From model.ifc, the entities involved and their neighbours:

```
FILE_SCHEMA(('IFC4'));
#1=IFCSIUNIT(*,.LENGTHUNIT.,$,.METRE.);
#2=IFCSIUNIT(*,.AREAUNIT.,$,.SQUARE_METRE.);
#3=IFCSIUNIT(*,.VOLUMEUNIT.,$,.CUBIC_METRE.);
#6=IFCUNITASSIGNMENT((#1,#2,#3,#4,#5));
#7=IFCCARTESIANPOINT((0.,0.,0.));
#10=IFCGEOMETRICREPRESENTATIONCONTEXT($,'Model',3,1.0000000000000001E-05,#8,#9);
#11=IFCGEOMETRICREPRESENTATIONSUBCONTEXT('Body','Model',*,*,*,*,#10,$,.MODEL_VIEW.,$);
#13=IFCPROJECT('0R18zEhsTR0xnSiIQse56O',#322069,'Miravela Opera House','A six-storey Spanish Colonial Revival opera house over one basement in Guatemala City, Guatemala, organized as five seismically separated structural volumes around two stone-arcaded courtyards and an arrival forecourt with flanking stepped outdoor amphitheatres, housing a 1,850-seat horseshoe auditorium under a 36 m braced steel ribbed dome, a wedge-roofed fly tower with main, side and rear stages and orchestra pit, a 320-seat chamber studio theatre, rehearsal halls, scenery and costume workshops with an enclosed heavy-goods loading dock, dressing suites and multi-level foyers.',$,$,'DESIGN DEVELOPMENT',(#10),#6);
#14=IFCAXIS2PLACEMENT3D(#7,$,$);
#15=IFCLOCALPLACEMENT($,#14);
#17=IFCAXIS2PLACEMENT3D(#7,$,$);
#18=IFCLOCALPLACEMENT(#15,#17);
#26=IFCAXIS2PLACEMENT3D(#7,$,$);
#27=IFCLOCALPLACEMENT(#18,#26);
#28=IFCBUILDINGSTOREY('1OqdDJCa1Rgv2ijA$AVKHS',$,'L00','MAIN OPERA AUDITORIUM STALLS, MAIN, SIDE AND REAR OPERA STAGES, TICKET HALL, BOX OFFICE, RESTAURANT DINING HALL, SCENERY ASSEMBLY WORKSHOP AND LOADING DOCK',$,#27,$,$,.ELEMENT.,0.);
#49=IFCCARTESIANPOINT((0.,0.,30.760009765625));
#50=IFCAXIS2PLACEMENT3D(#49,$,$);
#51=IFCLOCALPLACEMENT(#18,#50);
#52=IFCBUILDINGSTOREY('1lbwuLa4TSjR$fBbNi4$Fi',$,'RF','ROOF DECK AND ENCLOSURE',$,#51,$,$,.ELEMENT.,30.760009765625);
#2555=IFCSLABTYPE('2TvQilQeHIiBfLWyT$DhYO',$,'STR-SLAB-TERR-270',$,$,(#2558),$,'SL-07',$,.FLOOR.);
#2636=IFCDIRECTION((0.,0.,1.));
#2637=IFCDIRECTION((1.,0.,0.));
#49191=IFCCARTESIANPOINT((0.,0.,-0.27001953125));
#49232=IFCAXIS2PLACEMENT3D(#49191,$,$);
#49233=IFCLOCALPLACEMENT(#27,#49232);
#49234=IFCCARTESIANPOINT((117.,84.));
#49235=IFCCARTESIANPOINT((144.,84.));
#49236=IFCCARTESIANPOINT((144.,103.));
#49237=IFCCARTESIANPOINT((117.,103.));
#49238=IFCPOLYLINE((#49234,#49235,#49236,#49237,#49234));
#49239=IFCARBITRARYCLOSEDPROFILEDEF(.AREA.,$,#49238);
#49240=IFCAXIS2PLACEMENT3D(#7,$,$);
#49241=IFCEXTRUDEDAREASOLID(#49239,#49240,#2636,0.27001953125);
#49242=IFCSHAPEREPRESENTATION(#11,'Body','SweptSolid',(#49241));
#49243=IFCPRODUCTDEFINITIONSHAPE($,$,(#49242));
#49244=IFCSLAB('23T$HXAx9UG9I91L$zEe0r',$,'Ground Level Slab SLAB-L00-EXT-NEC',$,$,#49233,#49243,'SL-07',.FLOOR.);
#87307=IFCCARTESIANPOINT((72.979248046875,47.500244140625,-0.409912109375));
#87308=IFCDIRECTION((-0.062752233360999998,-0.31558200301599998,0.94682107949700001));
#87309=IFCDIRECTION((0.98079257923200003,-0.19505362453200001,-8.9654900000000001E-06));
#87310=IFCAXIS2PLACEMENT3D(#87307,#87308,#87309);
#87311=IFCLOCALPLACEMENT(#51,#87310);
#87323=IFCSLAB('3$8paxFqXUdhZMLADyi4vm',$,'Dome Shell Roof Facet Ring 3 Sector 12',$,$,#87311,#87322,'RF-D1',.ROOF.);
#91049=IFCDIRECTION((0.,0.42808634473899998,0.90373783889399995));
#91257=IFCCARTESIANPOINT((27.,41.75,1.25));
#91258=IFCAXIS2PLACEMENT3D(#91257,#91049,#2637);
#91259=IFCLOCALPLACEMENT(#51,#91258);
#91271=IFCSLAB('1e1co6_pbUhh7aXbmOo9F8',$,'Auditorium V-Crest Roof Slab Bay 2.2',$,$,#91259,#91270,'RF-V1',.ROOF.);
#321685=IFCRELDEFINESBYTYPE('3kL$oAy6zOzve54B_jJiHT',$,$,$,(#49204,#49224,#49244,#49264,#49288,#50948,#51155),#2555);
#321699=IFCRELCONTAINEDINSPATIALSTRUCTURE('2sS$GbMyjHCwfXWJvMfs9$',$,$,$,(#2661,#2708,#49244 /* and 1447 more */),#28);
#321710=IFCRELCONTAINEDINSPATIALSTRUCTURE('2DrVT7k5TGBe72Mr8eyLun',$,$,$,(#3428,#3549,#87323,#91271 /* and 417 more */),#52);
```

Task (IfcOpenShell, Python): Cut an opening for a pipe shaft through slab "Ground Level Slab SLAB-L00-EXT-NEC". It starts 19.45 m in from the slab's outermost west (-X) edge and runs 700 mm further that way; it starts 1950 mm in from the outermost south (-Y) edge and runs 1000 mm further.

```python
import numpy as np
import ifcopenshell
import ifcopenshell.api.feature
import ifcopenshell.api.geometry
import ifcopenshell.api.root
import ifcopenshell.geom
import ifcopenshell.util.placement
import ifcopenshell.util.representation
import ifcopenshell.util.shape
import ifcopenshell.util.unit

model = ifcopenshell.open("model.ifc")
unit_scale = ifcopenshell.util.unit.calculate_unit_scale(model)
settings = ifcopenshell.geom.settings()


def volume(element):
    """Net volume in cubic metres, openings subtracted."""
    shape = ifcopenshell.geom.create_shape(settings, element)
    return ifcopenshell.util.shape.get_volume(shape.geometry)


slab = model.by_guid("23T$HXAx9UG9I91L$zEe0r")
before = volume(slab)

# Extent in the slab's own axes, in metres. The edges named are its -X and -Y sides.
slab_shape = ifcopenshell.geom.create_shape(settings, slab)
vertices = ifcopenshell.util.shape.get_vertices(slab_shape.geometry)
x_min, y_min, bottom = vertices.min(axis=0)
top = vertices[:, 2].max()

opening = ifcopenshell.api.root.create_entity(model, ifc_class="IfcOpeningElement", name="Pipe shaft opening", predefined_type="OPENING")
context = ifcopenshell.util.representation.get_context(model, "Model", "Body", "MODEL_VIEW")
width, depth = 0.7, 1
outline = [(0.0, 0.0), (width, 0.0), (width, depth), (0.0, depth), (0.0, 0.0)]
# Overshoot both faces by 50 mm so the cut is clean.
shape = ifcopenshell.api.geometry.add_slab_representation(
    model, context=context, depth=top - bottom + 0.1, polyline=outline
)
ifcopenshell.api.geometry.assign_representation(model, product=opening, representation=shape)

matrix = ifcopenshell.util.placement.get_local_placement(slab.ObjectPlacement)
matrix[:, 3] = matrix @ np.append(np.array([x_min + 19.45, y_min + 1.95, bottom - 0.05]) / unit_scale, 1.0)
ifcopenshell.api.geometry.edit_object_placement(model, product=opening, matrix=matrix, is_si=False)
ifcopenshell.api.feature.add_feature(model, feature=opening, element=slab)

after = volume(slab)

print(f"slab volume {before:.3f} -> {after:.3f} m3")

model.write("model_edited.ifc")
```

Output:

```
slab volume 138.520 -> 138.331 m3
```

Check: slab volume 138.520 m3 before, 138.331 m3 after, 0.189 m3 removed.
